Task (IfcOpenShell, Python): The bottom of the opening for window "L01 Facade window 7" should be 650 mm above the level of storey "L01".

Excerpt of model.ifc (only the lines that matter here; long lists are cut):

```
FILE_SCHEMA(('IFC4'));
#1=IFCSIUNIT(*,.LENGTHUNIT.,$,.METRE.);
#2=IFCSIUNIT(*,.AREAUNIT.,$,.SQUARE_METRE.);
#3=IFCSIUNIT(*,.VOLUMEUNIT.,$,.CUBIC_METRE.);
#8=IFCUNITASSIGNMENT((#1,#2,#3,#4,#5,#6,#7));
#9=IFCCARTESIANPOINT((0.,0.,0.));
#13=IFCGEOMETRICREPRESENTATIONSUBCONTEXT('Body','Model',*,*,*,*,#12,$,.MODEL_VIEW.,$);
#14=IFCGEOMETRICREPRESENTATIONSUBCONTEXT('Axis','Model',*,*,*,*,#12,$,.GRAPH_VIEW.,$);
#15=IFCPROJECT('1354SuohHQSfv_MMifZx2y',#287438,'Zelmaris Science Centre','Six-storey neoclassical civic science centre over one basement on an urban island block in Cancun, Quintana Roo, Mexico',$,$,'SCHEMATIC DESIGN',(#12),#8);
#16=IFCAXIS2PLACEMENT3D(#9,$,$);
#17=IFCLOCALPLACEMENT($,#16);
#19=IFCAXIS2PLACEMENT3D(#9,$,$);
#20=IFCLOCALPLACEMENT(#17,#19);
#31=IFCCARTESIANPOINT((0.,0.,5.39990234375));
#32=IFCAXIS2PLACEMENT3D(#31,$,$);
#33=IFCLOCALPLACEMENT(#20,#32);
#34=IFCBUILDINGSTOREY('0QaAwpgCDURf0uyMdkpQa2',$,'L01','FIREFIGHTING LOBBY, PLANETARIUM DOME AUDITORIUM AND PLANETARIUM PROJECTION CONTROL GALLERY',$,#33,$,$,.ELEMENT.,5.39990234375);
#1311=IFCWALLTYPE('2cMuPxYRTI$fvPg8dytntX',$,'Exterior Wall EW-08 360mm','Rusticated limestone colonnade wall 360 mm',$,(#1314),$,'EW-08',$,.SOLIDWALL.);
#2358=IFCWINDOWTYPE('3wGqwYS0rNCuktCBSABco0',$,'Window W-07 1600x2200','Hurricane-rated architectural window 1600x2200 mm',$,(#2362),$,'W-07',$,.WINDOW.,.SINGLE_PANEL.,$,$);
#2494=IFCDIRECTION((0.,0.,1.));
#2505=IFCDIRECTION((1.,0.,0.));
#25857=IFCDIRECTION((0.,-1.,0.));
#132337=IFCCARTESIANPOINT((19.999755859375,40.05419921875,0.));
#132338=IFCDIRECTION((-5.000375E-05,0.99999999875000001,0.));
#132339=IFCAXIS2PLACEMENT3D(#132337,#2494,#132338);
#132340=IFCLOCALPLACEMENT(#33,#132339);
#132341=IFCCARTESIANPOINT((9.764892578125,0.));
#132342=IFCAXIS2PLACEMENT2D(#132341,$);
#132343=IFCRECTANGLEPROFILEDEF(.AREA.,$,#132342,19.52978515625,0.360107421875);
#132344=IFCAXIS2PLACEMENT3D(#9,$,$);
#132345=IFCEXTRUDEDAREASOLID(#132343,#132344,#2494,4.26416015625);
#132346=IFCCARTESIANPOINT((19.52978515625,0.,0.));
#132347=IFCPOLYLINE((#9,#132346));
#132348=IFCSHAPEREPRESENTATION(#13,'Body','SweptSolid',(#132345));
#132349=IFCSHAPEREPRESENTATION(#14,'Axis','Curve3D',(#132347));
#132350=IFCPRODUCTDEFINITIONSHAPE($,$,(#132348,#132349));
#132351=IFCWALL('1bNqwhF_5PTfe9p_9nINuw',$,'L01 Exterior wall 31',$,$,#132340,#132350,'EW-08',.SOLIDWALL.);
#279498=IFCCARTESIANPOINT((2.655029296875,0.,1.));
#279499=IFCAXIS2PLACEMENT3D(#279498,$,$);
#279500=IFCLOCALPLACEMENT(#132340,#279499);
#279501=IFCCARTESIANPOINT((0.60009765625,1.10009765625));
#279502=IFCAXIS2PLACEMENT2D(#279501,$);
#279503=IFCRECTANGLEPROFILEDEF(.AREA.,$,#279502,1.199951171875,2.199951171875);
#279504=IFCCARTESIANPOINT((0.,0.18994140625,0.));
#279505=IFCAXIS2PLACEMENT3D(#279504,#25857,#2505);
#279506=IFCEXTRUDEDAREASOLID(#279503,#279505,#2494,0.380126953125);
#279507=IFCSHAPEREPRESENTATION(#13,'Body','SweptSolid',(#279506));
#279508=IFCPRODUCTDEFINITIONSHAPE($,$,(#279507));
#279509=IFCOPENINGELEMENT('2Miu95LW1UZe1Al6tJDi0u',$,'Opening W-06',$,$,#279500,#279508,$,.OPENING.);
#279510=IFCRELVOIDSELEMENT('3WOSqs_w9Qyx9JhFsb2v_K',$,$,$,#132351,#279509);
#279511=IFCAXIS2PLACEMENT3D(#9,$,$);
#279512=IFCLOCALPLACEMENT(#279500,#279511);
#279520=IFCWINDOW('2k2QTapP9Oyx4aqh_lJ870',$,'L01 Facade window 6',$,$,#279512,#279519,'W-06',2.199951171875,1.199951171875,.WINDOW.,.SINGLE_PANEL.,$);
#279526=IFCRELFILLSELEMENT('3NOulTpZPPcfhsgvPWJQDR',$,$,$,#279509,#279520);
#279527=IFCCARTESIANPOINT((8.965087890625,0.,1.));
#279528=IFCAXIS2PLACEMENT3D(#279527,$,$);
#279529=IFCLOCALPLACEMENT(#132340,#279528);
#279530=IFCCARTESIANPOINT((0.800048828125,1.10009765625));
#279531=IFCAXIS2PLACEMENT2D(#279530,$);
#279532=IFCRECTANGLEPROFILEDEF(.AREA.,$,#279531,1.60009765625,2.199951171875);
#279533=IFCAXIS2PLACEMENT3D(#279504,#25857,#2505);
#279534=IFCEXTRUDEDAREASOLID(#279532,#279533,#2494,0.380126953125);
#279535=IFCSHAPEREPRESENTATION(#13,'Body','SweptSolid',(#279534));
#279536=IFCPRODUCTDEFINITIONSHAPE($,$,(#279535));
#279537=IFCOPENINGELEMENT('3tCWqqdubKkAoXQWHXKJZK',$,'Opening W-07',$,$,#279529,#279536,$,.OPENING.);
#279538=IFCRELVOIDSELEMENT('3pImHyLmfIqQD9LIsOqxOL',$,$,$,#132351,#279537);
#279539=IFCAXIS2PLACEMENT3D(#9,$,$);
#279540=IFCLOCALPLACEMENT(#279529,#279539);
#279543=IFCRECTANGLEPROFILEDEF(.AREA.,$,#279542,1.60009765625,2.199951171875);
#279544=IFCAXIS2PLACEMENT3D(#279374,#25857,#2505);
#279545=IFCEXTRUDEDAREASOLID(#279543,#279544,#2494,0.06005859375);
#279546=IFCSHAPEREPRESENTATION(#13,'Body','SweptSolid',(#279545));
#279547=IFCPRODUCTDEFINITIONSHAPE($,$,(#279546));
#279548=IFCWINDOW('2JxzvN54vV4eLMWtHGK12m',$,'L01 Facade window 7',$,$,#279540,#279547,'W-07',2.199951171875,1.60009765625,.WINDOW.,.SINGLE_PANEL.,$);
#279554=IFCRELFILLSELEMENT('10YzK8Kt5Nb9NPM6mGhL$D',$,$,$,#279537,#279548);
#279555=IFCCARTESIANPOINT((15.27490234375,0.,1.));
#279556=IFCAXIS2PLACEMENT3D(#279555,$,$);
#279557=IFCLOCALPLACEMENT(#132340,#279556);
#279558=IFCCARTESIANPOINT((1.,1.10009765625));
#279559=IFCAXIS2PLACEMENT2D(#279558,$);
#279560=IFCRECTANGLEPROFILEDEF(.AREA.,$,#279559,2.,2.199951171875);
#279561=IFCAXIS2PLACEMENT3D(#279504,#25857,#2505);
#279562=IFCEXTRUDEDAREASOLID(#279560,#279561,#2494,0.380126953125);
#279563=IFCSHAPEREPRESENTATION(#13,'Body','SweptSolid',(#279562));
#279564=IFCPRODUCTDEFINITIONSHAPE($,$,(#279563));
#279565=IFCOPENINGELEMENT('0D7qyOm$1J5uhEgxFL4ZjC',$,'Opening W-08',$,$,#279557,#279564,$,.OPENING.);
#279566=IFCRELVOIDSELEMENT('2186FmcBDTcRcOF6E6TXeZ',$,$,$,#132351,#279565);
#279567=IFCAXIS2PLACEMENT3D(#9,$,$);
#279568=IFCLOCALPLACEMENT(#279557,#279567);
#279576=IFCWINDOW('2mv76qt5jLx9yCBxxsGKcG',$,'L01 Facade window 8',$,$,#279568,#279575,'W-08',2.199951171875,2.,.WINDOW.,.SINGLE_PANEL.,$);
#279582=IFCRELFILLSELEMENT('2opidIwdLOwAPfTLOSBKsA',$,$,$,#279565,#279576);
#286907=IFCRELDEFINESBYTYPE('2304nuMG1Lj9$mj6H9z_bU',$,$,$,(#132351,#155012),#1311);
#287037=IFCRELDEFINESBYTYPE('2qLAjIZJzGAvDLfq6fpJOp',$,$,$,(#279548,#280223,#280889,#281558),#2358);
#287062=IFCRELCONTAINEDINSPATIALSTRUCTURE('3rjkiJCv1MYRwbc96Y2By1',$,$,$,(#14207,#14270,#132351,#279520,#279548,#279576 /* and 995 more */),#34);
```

```python
import numpy as np
import ifcopenshell
import ifcopenshell.api.geometry
import ifcopenshell.geom
import ifcopenshell.util.element
import ifcopenshell.util.placement
import ifcopenshell.util.shape
import ifcopenshell.util.unit

model = ifcopenshell.open("model.ifc")
unit_scale = ifcopenshell.util.unit.calculate_unit_scale(model)

window = model.by_id(279548)
opening = window.FillsVoids[0].RelatingOpeningElement
storey = ifcopenshell.util.element.get_container(window, ifc_class="IfcBuildingStorey")
level = ifcopenshell.util.placement.get_local_placement(storey.ObjectPlacement)[2, 3]

# The opening's origin need not be at the sill, so measure its lowest point.
shape = ifcopenshell.geom.create_shape(ifcopenshell.geom.settings(), opening)
bottom = ifcopenshell.util.shape.get_shape_bottom_elevation(shape, shape.geometry) / unit_scale
dz = level + 0.65 / unit_scale - bottom

shift = np.array([0.0, 0.0, dz])
# The window is placed relative to its opening, so it follows when the opening moves.
matrix = ifcopenshell.util.placement.get_local_placement(opening.ObjectPlacement)
matrix[:3, 3] += shift
ifcopenshell.api.geometry.edit_object_placement(
    model, product=opening, matrix=matrix, is_si=False, should_transform_children=True
)

print(f"moved by {dz * unit_scale:+.3f} m")

model.write("model_rev.ifc")
```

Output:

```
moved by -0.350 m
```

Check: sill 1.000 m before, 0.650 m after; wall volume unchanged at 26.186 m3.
